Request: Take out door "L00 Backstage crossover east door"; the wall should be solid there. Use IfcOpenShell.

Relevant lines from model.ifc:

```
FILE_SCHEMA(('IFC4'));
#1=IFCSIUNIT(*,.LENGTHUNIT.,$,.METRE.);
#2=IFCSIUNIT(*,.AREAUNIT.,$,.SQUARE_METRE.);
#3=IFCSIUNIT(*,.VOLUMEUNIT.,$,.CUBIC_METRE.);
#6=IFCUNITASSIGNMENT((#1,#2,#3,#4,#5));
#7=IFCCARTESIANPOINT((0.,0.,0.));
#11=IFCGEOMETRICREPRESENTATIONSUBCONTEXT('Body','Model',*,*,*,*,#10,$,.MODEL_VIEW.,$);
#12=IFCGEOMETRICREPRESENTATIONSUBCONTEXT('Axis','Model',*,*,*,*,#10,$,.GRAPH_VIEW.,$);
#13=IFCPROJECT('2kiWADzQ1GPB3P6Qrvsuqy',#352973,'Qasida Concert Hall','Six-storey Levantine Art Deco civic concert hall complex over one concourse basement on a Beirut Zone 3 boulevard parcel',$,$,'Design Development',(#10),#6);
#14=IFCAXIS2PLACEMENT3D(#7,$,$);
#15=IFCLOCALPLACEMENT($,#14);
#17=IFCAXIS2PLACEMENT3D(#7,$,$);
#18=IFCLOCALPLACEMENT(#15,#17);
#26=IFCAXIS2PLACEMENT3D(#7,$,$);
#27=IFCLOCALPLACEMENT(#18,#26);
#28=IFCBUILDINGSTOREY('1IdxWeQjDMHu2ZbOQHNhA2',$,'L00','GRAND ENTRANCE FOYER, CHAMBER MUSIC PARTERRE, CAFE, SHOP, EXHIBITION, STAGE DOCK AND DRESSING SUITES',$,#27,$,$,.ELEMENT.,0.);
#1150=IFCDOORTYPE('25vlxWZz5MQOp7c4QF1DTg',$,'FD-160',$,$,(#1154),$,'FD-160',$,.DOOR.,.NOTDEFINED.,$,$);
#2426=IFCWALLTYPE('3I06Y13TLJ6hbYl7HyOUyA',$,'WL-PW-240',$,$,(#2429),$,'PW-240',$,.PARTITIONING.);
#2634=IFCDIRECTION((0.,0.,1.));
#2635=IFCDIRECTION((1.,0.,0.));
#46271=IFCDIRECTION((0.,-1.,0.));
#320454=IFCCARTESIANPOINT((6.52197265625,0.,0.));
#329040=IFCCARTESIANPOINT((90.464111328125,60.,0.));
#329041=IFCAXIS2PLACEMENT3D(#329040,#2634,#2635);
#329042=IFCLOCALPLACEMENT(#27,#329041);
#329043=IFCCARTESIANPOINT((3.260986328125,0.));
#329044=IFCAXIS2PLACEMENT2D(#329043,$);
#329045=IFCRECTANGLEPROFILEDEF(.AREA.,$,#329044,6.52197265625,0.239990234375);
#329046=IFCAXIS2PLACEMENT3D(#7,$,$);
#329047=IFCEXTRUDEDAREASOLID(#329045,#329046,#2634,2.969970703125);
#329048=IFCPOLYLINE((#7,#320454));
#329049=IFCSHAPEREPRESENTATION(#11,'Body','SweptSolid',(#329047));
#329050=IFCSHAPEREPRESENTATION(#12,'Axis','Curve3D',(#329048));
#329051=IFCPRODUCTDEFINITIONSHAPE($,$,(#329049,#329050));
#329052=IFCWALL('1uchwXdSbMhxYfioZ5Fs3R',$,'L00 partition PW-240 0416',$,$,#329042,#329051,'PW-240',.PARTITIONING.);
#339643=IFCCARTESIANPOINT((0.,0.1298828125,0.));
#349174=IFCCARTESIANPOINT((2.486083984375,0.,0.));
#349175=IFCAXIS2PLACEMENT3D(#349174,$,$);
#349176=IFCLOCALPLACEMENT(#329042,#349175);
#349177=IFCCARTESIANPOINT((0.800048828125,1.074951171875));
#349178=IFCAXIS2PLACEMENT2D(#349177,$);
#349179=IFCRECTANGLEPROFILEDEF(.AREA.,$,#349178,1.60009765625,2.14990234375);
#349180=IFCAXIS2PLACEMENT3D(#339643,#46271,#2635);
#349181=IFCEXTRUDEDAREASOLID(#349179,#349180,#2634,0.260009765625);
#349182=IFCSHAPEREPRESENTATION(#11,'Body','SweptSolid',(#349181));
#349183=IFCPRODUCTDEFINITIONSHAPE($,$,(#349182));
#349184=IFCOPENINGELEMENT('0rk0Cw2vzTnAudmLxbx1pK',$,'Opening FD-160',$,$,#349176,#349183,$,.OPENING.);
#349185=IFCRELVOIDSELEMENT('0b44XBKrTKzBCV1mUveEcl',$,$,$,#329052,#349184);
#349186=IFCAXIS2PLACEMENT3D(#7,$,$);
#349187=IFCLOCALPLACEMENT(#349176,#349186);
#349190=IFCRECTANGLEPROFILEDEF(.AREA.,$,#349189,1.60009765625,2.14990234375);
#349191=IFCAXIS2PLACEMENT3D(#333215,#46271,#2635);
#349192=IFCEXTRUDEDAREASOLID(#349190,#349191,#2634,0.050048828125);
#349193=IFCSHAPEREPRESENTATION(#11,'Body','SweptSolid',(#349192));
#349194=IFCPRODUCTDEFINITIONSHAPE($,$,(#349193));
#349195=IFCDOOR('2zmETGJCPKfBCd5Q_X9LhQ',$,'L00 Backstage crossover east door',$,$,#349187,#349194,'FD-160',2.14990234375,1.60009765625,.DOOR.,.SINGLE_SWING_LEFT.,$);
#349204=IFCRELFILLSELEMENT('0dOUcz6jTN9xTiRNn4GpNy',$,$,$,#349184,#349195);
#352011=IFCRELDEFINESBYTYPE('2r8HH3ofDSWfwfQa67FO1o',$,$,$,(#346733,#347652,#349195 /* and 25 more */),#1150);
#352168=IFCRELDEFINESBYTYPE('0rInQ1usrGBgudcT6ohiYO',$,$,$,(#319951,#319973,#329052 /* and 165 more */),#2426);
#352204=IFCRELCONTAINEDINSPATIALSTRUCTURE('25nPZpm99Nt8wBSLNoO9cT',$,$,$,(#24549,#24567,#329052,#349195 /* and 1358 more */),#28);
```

```python
import ifcopenshell
import ifcopenshell.api.feature
import ifcopenshell.api.root
import ifcopenshell.geom
import ifcopenshell.util.shape

model = ifcopenshell.open("model.ifc")
settings = ifcopenshell.geom.settings()


def volume(element):
    """Net volume in cubic metres, openings subtracted."""
    shape = ifcopenshell.geom.create_shape(settings, element)
    return ifcopenshell.util.shape.get_volume(shape.geometry)


door = model.by_guid("2zmETGJCPKfBCd5Q_X9LhQ")
opening = door.FillsVoids[0].RelatingOpeningElement
wall = opening.VoidsElements[0].RelatingBuildingElement
before = volume(wall)

ifcopenshell.api.root.remove_product(model, product=door)
ifcopenshell.api.feature.remove_feature(model, feature=opening)

after = volume(wall)

print(f"wall volume {before:.3f} -> {after:.3f} m3")

model.write("model_updated.ifc")
```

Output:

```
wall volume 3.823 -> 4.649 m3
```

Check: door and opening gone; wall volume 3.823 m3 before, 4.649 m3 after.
